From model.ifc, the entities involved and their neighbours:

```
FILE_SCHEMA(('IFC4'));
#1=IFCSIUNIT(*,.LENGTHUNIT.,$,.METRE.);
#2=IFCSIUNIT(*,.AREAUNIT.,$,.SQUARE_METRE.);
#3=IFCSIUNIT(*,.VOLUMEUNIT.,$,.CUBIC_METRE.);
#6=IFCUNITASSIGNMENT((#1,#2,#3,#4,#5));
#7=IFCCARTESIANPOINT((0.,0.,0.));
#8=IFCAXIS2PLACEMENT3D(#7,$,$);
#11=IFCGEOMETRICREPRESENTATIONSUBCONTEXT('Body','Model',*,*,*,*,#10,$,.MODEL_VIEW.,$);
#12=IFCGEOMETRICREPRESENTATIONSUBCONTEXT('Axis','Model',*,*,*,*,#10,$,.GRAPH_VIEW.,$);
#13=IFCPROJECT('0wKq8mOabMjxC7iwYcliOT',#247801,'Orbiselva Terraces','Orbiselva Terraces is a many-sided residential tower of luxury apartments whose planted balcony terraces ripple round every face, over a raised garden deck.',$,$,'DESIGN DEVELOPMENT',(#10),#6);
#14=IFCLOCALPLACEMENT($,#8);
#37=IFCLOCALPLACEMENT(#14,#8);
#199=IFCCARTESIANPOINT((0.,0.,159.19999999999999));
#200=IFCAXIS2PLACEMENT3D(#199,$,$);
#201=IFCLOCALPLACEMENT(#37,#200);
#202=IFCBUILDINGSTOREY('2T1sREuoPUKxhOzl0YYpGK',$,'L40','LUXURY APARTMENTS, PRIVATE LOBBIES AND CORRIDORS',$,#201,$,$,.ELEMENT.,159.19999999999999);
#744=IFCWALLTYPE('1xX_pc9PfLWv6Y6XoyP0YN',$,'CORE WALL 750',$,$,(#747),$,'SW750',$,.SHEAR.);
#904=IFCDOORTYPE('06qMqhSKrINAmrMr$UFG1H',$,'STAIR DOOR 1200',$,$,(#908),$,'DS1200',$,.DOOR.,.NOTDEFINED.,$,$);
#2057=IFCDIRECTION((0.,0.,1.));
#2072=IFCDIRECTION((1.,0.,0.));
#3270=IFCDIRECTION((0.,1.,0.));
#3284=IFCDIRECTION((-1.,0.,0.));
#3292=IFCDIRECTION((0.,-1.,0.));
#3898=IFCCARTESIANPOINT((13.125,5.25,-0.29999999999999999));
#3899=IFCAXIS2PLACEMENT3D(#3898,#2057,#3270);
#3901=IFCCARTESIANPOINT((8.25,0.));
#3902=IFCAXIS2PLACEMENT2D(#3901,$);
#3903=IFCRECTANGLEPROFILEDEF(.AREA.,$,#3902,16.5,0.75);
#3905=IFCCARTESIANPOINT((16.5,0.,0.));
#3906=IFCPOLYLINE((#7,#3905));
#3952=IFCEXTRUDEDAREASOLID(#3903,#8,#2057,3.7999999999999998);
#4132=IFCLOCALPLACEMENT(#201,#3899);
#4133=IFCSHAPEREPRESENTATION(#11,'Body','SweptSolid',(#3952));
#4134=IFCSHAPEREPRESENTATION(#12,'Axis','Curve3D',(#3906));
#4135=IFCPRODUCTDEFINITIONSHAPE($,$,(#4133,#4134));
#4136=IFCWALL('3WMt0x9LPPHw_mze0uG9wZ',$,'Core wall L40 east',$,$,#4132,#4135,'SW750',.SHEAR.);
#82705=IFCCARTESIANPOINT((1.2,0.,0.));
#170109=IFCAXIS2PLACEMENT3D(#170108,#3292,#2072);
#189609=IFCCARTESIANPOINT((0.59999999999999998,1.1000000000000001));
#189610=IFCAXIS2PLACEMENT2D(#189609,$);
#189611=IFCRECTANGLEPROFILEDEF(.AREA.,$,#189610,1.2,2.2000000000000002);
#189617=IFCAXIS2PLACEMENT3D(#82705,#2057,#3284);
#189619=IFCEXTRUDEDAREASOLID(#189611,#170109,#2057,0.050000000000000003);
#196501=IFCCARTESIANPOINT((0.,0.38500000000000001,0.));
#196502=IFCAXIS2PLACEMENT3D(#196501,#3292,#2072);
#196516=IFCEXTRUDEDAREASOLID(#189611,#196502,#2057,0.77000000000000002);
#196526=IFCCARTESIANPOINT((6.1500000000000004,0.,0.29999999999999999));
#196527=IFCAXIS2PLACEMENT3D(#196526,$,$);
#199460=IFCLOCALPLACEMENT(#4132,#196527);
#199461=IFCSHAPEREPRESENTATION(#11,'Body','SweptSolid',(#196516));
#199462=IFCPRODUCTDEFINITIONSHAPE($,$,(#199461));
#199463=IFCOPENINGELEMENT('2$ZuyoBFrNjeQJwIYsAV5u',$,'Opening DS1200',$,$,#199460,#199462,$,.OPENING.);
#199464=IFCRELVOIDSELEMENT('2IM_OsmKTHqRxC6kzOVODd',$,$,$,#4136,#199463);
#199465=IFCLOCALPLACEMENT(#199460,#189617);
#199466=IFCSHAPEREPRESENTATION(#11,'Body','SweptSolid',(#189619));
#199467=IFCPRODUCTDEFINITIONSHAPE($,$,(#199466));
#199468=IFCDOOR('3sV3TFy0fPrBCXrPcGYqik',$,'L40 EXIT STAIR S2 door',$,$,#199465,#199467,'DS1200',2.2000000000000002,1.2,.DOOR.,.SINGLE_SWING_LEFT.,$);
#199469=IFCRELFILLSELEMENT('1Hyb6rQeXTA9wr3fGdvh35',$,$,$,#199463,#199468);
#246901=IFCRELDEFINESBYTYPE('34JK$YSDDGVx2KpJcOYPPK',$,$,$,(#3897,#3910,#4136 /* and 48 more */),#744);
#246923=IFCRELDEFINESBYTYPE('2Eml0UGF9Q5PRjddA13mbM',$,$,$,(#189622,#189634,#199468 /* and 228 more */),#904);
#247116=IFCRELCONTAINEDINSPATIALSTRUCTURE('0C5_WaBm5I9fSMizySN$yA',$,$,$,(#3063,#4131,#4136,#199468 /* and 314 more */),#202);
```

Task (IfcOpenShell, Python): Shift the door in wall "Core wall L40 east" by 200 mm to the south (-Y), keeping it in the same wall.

```python
import ifcopenshell
import ifcopenshell.api.geometry
import ifcopenshell.util.placement

model = ifcopenshell.open("model.ifc")

door = model.by_guid("3sV3TFy0fPrBCXrPcGYqik")
opening = door.FillsVoids[0].RelatingOpeningElement
wall = opening.VoidsElements[0].RelatingBuildingElement

wall_matrix = ifcopenshell.util.placement.get_local_placement(wall.ObjectPlacement)
shift = wall_matrix[:3, 0] * -0.2
before = ifcopenshell.util.placement.get_local_placement(door.ObjectPlacement)[:3, 3].copy()

# The door is placed relative to its opening, so it follows when the opening moves.
matrix = ifcopenshell.util.placement.get_local_placement(opening.ObjectPlacement)
matrix[:3, 3] += shift
ifcopenshell.api.geometry.edit_object_placement(
    model, product=opening, matrix=matrix, is_si=False, should_transform_children=True
)

after = ifcopenshell.util.placement.get_local_placement(door.ObjectPlacement)[:3, 3]
print("door moved by", (after - before).round(3) + 0.0)

model.write("model_v2.ifc")
```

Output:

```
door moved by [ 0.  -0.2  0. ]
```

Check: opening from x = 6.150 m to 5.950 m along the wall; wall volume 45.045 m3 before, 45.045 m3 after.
